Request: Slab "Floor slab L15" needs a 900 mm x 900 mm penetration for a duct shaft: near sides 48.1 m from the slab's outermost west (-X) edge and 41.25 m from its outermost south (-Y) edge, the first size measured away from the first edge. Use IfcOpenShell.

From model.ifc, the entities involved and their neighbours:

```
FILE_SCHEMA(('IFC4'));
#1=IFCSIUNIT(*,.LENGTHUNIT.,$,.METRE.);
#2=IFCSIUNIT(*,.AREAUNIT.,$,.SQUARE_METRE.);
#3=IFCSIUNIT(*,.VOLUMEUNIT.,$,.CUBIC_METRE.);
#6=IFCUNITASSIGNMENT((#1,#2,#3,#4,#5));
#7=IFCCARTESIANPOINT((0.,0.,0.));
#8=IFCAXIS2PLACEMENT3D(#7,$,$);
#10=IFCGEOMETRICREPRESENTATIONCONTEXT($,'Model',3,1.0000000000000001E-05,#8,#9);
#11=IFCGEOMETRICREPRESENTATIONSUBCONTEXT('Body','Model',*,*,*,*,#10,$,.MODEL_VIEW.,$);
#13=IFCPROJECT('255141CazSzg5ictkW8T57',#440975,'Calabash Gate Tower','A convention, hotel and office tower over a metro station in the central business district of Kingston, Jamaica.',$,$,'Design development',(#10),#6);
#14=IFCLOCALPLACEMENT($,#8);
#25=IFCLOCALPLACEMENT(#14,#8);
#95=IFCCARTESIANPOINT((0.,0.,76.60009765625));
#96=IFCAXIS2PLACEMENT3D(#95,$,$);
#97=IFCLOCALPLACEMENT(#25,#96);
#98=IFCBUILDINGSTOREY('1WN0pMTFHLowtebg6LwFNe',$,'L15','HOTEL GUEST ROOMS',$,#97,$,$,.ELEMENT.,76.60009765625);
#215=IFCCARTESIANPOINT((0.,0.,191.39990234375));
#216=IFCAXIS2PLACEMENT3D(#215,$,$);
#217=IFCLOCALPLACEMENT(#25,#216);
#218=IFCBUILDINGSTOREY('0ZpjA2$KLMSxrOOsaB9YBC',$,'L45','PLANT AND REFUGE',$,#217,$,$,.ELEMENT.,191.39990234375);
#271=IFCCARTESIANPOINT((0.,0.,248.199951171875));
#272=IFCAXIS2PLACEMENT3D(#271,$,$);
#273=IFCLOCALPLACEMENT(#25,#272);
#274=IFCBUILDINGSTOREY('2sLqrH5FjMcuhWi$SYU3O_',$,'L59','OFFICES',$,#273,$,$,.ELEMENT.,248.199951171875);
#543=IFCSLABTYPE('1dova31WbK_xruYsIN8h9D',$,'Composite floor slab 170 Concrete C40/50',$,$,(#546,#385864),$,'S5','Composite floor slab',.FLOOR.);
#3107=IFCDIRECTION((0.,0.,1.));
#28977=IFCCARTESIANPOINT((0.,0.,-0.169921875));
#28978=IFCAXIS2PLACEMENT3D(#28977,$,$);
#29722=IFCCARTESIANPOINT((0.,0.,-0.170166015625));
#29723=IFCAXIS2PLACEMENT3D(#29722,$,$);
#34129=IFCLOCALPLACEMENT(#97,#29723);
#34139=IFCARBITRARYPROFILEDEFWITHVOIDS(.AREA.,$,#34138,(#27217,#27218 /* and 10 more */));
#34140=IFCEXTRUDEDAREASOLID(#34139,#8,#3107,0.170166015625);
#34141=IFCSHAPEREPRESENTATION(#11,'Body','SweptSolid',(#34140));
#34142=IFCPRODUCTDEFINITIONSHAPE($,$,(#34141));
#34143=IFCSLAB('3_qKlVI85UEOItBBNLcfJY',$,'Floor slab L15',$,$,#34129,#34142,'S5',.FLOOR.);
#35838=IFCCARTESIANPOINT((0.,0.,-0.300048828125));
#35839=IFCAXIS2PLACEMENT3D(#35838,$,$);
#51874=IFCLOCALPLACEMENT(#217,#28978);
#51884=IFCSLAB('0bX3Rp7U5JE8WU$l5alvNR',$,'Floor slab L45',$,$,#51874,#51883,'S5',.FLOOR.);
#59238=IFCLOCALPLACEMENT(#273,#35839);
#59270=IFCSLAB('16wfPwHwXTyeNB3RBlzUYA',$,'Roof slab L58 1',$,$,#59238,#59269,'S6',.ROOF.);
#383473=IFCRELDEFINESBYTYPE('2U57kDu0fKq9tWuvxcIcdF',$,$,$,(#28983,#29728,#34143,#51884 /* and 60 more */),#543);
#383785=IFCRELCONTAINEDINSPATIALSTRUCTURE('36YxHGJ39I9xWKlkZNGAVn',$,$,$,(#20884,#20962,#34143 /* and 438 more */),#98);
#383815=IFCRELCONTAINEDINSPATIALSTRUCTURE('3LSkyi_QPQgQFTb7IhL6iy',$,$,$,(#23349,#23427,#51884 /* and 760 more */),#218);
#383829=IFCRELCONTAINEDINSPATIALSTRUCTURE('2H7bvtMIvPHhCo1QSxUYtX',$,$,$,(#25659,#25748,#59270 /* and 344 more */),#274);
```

```python
import numpy as np
import ifcopenshell
import ifcopenshell.api.feature
import ifcopenshell.api.geometry
import ifcopenshell.api.root
import ifcopenshell.geom
import ifcopenshell.util.placement
import ifcopenshell.util.representation
import ifcopenshell.util.shape
import ifcopenshell.util.unit

model = ifcopenshell.open("model.ifc")
unit_scale = ifcopenshell.util.unit.calculate_unit_scale(model)
settings = ifcopenshell.geom.settings()


def volume(element):
    """Net volume in cubic metres, openings subtracted."""
    shape = ifcopenshell.geom.create_shape(settings, element)
    return ifcopenshell.util.shape.get_volume(shape.geometry)


slab = model.by_guid("3_qKlVI85UEOItBBNLcfJY")
before = volume(slab)

# Extent in the slab's own axes, in metres. The edges named are its -X and -Y sides.
slab_shape = ifcopenshell.geom.create_shape(settings, slab)
vertices = ifcopenshell.util.shape.get_vertices(slab_shape.geometry)
x_min, y_min, bottom = vertices.min(axis=0)
top = vertices[:, 2].max()

opening = ifcopenshell.api.root.create_entity(model, ifc_class="IfcOpeningElement", name="Duct shaft opening", predefined_type="OPENING")
context = ifcopenshell.util.representation.get_context(model, "Model", "Body", "MODEL_VIEW")
width, depth = 0.9, 0.9
outline = [(0.0, 0.0), (width, 0.0), (width, depth), (0.0, depth), (0.0, 0.0)]
# Overshoot both faces by 50 mm so the cut is clean.
shape = ifcopenshell.api.geometry.add_slab_representation(
    model, context=context, depth=top - bottom + 0.1, polyline=outline
)
ifcopenshell.api.geometry.assign_representation(model, product=opening, representation=shape)

matrix = ifcopenshell.util.placement.get_local_placement(slab.ObjectPlacement)
matrix[:, 3] = matrix @ np.append(np.array([x_min + 48.1, y_min + 41.25, bottom - 0.05]) / unit_scale, 1.0)
ifcopenshell.api.geometry.edit_object_placement(model, product=opening, matrix=matrix, is_si=False)
ifcopenshell.api.feature.add_feature(model, feature=opening, element=slab)

after = volume(slab)

print(f"slab volume {before:.3f} -> {after:.3f} m3")

model.write("model-out.ifc")
```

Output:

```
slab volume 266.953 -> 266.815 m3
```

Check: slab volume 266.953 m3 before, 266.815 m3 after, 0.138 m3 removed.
